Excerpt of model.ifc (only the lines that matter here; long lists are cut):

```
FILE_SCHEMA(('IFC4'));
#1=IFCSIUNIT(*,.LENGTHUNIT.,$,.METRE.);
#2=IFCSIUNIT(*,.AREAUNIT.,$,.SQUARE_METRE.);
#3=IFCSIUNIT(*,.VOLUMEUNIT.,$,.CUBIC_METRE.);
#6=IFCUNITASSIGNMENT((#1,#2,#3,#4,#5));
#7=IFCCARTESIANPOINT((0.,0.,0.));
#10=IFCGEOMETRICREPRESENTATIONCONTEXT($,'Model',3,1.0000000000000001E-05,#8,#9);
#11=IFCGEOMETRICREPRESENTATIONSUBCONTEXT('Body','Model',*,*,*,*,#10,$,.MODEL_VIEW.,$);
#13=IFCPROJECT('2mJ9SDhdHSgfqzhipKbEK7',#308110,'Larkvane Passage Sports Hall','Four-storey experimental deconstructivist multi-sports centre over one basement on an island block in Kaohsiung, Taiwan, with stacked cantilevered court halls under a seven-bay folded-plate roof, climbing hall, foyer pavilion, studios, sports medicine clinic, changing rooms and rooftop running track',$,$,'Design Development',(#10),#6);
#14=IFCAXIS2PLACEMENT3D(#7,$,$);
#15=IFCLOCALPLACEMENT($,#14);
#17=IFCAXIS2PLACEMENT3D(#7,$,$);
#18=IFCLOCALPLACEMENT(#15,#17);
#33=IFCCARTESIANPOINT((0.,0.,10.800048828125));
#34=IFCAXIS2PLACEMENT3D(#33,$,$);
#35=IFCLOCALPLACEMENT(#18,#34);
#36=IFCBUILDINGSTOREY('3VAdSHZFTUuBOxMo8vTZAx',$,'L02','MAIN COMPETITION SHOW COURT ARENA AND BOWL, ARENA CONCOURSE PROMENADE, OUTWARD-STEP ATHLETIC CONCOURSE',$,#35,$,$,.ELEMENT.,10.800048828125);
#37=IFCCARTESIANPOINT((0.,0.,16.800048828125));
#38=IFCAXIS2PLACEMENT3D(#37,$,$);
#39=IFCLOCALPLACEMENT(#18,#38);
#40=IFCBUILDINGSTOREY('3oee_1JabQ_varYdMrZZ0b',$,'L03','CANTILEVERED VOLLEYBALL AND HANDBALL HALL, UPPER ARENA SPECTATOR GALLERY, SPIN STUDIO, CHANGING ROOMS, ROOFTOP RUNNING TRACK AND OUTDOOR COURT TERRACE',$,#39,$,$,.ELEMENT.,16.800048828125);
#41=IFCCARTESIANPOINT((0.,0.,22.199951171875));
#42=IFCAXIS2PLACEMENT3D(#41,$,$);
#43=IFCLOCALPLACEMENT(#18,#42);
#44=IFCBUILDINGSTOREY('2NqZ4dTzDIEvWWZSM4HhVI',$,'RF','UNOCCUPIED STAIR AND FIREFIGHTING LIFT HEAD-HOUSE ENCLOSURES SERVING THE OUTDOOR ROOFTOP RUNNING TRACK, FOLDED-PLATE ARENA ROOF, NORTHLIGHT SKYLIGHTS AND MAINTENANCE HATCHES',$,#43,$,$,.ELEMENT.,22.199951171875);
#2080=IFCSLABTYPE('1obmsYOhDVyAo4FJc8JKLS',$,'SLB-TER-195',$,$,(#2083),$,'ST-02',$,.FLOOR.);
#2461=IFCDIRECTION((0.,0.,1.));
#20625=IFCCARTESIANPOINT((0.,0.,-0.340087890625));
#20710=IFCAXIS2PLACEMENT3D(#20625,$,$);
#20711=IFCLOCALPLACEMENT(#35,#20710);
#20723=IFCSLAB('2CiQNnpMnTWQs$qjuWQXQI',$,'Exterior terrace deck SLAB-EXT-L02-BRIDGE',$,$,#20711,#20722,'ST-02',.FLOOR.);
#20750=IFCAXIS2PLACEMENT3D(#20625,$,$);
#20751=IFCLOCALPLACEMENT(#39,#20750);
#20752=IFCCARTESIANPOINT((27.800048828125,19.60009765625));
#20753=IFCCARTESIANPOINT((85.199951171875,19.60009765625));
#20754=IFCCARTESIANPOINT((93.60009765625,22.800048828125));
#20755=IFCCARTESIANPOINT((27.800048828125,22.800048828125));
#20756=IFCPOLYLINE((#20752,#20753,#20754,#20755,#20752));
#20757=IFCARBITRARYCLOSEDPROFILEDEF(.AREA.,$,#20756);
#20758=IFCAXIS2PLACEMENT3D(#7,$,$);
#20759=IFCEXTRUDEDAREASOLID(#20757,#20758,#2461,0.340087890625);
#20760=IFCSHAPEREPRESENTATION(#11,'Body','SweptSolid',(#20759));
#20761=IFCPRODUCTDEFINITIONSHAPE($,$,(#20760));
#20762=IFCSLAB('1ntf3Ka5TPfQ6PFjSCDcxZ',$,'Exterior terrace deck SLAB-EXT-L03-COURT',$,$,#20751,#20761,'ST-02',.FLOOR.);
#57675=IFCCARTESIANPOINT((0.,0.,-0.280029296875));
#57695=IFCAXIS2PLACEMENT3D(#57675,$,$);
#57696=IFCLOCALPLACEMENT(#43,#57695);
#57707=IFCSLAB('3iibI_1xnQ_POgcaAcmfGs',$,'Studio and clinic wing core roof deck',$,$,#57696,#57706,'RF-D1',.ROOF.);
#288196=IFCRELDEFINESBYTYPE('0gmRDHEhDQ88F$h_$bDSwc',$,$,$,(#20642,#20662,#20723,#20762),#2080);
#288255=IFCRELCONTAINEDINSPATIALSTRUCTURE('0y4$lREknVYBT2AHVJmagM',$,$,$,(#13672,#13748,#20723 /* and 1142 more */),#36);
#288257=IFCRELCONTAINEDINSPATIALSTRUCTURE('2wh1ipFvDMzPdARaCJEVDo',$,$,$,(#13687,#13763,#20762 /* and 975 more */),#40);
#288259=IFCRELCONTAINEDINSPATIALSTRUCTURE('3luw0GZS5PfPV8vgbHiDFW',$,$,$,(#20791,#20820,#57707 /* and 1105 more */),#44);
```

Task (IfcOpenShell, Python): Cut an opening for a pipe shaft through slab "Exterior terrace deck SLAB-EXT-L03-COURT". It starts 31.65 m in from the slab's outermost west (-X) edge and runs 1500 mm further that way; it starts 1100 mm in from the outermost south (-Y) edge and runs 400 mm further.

```python
import numpy as np
import ifcopenshell
import ifcopenshell.api.feature
import ifcopenshell.api.geometry
import ifcopenshell.api.root
import ifcopenshell.geom
import ifcopenshell.util.placement
import ifcopenshell.util.representation
import ifcopenshell.util.shape
import ifcopenshell.util.unit

model = ifcopenshell.open("model.ifc")
unit_scale = ifcopenshell.util.unit.calculate_unit_scale(model)
settings = ifcopenshell.geom.settings()


def volume(element):
    """Net volume in cubic metres, openings subtracted."""
    shape = ifcopenshell.geom.create_shape(settings, element)
    return ifcopenshell.util.shape.get_volume(shape.geometry)


slab = model.by_id(20762)
before = volume(slab)

# Extent in the slab's own axes, in metres. The edges named are its -X and -Y sides.
slab_shape = ifcopenshell.geom.create_shape(settings, slab)
vertices = ifcopenshell.util.shape.get_vertices(slab_shape.geometry)
x_min, y_min, bottom = vertices.min(axis=0)
top = vertices[:, 2].max()

opening = ifcopenshell.api.root.create_entity(model, ifc_class="IfcOpeningElement", name="Pipe shaft opening", predefined_type="OPENING")
context = ifcopenshell.util.representation.get_context(model, "Model", "Body", "MODEL_VIEW")
width, depth = 1.5, 0.4
outline = [(0.0, 0.0), (width, 0.0), (width, depth), (0.0, depth), (0.0, 0.0)]
# Overshoot both faces by 50 mm so the cut is clean.
shape = ifcopenshell.api.geometry.add_slab_representation(
    model, context=context, depth=top - bottom + 0.1, polyline=outline
)
ifcopenshell.api.geometry.assign_representation(model, product=opening, representation=shape)

matrix = ifcopenshell.util.placement.get_local_placement(slab.ObjectPlacement)
matrix[:, 3] = matrix @ np.append(np.array([x_min + 31.65, y_min + 1.1, bottom - 0.05]) / unit_scale, 1.0)
ifcopenshell.api.geometry.edit_object_placement(model, product=opening, matrix=matrix, is_si=False)
ifcopenshell.api.feature.add_feature(model, feature=opening, element=slab)

after = volume(slab)

print(f"slab volume {before:.3f} -> {after:.3f} m3")

model.write("model-out.ifc")
```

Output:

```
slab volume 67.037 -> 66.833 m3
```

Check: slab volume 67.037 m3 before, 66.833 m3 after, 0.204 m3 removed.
